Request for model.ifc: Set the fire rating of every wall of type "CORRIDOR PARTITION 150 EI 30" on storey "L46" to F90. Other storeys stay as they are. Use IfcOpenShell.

First a look at what the model holds.

```python
import ifcopenshell
import ifcopenshell.util.element

model = ifcopenshell.open("model.ifc")
print(model.schema)
storey = next(s for s in model.by_type("IfcBuildingStorey") if s.Name == "L46")
walls = [e for e in ifcopenshell.util.element.get_decomposition(storey) if e.is_a("IfcWall")]
seen = {}
for e in walls:
    element_type = ifcopenshell.util.element.get_type(e)
    key = (element_type.Name if element_type != e and element_type else None, ifcopenshell.util.element.get_pset(e, "Pset_WallCommon", "FireRating"))
    seen[key] = seen.get(key, 0) + 1
for (name, value), count in sorted(seen.items(), key=str):
    print(count, "x", name, "|", value)
```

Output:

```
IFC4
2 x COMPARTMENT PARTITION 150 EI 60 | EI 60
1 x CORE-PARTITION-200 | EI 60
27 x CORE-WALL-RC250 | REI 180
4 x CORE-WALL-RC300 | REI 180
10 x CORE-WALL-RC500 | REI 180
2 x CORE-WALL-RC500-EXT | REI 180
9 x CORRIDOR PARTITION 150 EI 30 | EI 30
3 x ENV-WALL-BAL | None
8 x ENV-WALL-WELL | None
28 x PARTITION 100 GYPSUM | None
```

```python
import ifcopenshell
import ifcopenshell.api.pset
import ifcopenshell.util.element

model = ifcopenshell.open("model.ifc")

storey = next(s for s in model.by_type("IfcBuildingStorey") if s.Name == "L46")
walls = [e for e in ifcopenshell.util.element.get_decomposition(storey) if e.is_a("IfcWall")]

count = 0
for e in walls:
    element_type = ifcopenshell.util.element.get_type(e)
    if element_type in (None, e) or element_type.Name != "CORRIDOR PARTITION 150 EI 30":
        continue
    found = ifcopenshell.util.element.get_pset(e, "Pset_WallCommon", should_inherit=False)
    if found:
        pset = model.by_id(found["id"])
        if len(ifcopenshell.util.element.get_elements_by_pset(pset)) > 1:
            pset = ifcopenshell.api.pset.unshare_pset(model, products=[e], pset=pset)[0]
    else:
        pset = ifcopenshell.api.pset.add_pset(model, product=e, name="Pset_WallCommon")
    ifcopenshell.api.pset.edit_pset(model, pset=pset, properties={"FireRating": "F90"})
    count += 1

print(count, "walls updated")

model.write("model_edited.ifc")
```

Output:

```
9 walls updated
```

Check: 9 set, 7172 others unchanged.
